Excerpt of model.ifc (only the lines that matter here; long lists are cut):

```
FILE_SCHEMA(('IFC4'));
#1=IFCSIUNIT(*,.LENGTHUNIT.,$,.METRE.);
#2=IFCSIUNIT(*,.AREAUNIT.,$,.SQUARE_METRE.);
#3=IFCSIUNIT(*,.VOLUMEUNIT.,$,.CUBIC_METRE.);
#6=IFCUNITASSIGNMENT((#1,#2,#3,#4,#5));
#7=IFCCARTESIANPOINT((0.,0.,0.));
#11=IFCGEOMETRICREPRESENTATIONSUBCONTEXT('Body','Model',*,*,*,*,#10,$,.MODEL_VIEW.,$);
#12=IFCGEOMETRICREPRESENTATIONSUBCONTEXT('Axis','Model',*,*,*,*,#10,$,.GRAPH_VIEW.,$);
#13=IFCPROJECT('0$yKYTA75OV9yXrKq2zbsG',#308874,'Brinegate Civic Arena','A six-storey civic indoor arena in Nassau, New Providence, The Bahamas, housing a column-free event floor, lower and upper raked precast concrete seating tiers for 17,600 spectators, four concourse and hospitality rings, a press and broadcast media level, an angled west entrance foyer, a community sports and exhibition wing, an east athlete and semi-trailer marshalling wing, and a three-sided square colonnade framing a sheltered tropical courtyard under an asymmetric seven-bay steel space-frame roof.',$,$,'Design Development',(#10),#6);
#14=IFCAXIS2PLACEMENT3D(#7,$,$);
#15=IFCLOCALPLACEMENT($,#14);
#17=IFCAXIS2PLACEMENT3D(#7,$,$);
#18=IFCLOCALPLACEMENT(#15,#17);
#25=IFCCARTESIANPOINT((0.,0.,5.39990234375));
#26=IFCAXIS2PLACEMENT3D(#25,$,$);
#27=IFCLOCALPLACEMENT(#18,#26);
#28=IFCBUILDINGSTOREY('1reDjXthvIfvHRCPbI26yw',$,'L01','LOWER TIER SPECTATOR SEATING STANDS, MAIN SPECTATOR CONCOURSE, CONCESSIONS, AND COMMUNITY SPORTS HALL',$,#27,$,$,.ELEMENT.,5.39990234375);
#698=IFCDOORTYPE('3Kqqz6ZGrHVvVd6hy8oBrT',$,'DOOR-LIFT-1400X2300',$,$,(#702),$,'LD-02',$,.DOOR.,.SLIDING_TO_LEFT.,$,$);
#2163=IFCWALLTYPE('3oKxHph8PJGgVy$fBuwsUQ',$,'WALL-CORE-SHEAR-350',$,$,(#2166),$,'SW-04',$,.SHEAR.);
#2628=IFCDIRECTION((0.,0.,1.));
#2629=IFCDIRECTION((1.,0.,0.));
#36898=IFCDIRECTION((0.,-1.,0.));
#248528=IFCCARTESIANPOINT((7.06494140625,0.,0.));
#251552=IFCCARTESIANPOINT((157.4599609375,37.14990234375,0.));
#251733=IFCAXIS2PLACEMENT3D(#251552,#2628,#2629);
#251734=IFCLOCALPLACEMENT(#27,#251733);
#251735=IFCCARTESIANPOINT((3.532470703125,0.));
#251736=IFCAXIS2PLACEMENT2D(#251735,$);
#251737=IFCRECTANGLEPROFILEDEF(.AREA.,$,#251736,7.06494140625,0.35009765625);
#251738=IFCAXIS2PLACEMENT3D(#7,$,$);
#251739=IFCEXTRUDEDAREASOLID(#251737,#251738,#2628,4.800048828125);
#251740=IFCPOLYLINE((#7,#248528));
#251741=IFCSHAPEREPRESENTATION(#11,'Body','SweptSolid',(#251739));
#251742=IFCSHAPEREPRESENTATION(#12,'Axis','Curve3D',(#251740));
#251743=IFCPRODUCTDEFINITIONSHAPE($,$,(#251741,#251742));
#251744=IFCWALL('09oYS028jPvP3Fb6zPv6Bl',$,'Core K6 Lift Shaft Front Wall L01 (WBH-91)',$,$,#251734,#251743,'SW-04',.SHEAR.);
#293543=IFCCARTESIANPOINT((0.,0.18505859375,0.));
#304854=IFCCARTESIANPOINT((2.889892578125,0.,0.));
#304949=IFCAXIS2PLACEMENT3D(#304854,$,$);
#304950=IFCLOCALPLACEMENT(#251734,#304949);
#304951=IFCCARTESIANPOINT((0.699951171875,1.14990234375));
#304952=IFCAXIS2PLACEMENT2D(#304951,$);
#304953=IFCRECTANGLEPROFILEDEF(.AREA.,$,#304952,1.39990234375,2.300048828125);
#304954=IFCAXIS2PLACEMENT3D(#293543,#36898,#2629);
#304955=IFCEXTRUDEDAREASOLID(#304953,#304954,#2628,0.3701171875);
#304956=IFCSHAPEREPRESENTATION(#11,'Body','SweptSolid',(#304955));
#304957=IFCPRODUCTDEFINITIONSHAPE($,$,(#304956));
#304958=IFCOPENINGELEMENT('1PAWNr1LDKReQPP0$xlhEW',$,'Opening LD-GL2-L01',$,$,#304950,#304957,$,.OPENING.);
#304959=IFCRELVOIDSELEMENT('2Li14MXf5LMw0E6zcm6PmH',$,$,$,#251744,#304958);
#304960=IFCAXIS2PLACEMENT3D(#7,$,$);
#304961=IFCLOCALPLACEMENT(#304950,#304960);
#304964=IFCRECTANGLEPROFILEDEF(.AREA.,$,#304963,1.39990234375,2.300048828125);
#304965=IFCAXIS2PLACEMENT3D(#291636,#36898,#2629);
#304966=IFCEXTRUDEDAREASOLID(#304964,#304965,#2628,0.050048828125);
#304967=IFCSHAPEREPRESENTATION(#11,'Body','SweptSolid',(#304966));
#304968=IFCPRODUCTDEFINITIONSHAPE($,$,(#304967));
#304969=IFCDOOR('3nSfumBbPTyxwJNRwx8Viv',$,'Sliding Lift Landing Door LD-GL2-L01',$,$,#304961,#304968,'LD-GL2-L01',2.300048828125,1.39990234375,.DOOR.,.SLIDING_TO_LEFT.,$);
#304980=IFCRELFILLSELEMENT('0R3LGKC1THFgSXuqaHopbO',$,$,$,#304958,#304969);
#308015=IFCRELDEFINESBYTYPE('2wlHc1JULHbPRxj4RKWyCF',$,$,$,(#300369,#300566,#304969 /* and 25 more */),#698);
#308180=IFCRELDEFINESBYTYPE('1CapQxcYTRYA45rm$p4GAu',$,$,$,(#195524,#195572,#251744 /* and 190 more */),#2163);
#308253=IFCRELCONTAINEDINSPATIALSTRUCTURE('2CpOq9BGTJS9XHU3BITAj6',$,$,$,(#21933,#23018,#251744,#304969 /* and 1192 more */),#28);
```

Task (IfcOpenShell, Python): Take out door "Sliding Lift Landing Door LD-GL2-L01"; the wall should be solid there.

```python
import ifcopenshell
import ifcopenshell.api.feature
import ifcopenshell.api.root
import ifcopenshell.geom
import ifcopenshell.util.shape

model = ifcopenshell.open("model.ifc")
settings = ifcopenshell.geom.settings()


def volume(element):
    """Net volume in cubic metres, openings subtracted."""
    shape = ifcopenshell.geom.create_shape(settings, element)
    return ifcopenshell.util.shape.get_volume(shape.geometry)


door = model.by_guid("3nSfumBbPTyxwJNRwx8Viv")
opening = door.FillsVoids[0].RelatingOpeningElement
wall = opening.VoidsElements[0].RelatingBuildingElement
before = volume(wall)

ifcopenshell.api.root.remove_product(model, product=door)
ifcopenshell.api.feature.remove_feature(model, feature=opening)

after = volume(wall)

print(f"wall volume {before:.3f} -> {after:.3f} m3")

model.write("model_edited.ifc")
```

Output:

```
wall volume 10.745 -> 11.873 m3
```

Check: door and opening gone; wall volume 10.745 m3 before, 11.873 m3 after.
